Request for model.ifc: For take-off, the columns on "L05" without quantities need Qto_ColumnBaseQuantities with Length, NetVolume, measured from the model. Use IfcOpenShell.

First a look at what the model holds.

```python
import ifcopenshell
import ifcopenshell.util.element
import ifcopenshell.util.unit

model = ifcopenshell.open("model.ifc")
print(model.schema)
for unit_type in ("LENGTHUNIT", "AREAUNIT", "VOLUMEUNIT"):
    print(unit_type, ifcopenshell.util.unit.calculate_unit_scale(model, unit_type))
storey = next(s for s in model.by_type("IfcBuildingStorey") if s.Name == "L05")
columns = [e for e in ifcopenshell.util.element.get_decomposition(storey) if e.is_a("IfcColumn")]
for e in sorted(columns, key=lambda e: e.id()):
    print(e.id(), e.is_a(), e.Name, list(ifcopenshell.util.element.get_psets(e, qtos_only=True)), sep=" | ")
```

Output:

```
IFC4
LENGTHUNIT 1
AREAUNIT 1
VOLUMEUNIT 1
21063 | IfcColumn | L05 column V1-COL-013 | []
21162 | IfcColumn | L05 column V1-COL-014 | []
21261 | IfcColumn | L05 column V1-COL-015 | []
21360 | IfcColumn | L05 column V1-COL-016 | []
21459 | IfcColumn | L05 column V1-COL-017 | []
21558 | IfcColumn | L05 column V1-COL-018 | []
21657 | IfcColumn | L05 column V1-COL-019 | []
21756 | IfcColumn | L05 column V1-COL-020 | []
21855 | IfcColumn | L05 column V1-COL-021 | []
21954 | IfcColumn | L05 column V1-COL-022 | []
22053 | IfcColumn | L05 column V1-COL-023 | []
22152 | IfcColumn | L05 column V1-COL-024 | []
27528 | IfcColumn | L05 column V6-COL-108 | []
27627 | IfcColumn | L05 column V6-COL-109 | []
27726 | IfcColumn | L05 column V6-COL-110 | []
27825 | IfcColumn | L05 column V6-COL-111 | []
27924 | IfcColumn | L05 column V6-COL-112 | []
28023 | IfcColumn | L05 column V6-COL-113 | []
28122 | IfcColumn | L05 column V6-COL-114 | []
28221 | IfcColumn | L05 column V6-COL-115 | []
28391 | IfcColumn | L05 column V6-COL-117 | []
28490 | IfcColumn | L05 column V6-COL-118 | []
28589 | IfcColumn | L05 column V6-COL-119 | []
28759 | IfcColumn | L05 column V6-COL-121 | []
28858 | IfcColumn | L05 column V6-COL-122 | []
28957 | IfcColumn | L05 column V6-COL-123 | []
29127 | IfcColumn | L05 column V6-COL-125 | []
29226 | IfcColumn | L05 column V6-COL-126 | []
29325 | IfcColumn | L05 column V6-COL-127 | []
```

```python
import ifcopenshell
import ifcopenshell.api.pset
import ifcopenshell.geom
import ifcopenshell.util.element
import ifcopenshell.util.shape
import ifcopenshell.util.unit

model = ifcopenshell.open("model.ifc")
unit_scale = ifcopenshell.util.unit.calculate_unit_scale(model)
volume_scale = ifcopenshell.util.unit.calculate_unit_scale(model, "VOLUMEUNIT")
settings = ifcopenshell.geom.settings()

storey = next(s for s in model.by_type("IfcBuildingStorey") if s.Name == "L05")
columns = [e for e in ifcopenshell.util.element.get_decomposition(storey) if e.is_a("IfcColumn")]

for e in sorted(columns, key=lambda e: e.id()):
    if ifcopenshell.util.element.get_psets(e, qtos_only=True, should_inherit=False):
        continue
    # Geometry comes back in metres, in the element's own axes.
    shape = ifcopenshell.geom.create_shape(settings, e)
    values = {
        "Length": ifcopenshell.util.shape.get_z(shape.geometry) / unit_scale,
        "NetVolume": ifcopenshell.util.shape.get_volume(shape.geometry) / volume_scale,
    }
    qto = ifcopenshell.api.pset.add_qto(model, product=e, name="Qto_ColumnBaseQuantities")
    ifcopenshell.api.pset.edit_qto(model, qto=qto, properties=values)
    print(e.id(), {k: round(v, 3) for k, v in values.items()})

model.write("model_edited.ifc")
```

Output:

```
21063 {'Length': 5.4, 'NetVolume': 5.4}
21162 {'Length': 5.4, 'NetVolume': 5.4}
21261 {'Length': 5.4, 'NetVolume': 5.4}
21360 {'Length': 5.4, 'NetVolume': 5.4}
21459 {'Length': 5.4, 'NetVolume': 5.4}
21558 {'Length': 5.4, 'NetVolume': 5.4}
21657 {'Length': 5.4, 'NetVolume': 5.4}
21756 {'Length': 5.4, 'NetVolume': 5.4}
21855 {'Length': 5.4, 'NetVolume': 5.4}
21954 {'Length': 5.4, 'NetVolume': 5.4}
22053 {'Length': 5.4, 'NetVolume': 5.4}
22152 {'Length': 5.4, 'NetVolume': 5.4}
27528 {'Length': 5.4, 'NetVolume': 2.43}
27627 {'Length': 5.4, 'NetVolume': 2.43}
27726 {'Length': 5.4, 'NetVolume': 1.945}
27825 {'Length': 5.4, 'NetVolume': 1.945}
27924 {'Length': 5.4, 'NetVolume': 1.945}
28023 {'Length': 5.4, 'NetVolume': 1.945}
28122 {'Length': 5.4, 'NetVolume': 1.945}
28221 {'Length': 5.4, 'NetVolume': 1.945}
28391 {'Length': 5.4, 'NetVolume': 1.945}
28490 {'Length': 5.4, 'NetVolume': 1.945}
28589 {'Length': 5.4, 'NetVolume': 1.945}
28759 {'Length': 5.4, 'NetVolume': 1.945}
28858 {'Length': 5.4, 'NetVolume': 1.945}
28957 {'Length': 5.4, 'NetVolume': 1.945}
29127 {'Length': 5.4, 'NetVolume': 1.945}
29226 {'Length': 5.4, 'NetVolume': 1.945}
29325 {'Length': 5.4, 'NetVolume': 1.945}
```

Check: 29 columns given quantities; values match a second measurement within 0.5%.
